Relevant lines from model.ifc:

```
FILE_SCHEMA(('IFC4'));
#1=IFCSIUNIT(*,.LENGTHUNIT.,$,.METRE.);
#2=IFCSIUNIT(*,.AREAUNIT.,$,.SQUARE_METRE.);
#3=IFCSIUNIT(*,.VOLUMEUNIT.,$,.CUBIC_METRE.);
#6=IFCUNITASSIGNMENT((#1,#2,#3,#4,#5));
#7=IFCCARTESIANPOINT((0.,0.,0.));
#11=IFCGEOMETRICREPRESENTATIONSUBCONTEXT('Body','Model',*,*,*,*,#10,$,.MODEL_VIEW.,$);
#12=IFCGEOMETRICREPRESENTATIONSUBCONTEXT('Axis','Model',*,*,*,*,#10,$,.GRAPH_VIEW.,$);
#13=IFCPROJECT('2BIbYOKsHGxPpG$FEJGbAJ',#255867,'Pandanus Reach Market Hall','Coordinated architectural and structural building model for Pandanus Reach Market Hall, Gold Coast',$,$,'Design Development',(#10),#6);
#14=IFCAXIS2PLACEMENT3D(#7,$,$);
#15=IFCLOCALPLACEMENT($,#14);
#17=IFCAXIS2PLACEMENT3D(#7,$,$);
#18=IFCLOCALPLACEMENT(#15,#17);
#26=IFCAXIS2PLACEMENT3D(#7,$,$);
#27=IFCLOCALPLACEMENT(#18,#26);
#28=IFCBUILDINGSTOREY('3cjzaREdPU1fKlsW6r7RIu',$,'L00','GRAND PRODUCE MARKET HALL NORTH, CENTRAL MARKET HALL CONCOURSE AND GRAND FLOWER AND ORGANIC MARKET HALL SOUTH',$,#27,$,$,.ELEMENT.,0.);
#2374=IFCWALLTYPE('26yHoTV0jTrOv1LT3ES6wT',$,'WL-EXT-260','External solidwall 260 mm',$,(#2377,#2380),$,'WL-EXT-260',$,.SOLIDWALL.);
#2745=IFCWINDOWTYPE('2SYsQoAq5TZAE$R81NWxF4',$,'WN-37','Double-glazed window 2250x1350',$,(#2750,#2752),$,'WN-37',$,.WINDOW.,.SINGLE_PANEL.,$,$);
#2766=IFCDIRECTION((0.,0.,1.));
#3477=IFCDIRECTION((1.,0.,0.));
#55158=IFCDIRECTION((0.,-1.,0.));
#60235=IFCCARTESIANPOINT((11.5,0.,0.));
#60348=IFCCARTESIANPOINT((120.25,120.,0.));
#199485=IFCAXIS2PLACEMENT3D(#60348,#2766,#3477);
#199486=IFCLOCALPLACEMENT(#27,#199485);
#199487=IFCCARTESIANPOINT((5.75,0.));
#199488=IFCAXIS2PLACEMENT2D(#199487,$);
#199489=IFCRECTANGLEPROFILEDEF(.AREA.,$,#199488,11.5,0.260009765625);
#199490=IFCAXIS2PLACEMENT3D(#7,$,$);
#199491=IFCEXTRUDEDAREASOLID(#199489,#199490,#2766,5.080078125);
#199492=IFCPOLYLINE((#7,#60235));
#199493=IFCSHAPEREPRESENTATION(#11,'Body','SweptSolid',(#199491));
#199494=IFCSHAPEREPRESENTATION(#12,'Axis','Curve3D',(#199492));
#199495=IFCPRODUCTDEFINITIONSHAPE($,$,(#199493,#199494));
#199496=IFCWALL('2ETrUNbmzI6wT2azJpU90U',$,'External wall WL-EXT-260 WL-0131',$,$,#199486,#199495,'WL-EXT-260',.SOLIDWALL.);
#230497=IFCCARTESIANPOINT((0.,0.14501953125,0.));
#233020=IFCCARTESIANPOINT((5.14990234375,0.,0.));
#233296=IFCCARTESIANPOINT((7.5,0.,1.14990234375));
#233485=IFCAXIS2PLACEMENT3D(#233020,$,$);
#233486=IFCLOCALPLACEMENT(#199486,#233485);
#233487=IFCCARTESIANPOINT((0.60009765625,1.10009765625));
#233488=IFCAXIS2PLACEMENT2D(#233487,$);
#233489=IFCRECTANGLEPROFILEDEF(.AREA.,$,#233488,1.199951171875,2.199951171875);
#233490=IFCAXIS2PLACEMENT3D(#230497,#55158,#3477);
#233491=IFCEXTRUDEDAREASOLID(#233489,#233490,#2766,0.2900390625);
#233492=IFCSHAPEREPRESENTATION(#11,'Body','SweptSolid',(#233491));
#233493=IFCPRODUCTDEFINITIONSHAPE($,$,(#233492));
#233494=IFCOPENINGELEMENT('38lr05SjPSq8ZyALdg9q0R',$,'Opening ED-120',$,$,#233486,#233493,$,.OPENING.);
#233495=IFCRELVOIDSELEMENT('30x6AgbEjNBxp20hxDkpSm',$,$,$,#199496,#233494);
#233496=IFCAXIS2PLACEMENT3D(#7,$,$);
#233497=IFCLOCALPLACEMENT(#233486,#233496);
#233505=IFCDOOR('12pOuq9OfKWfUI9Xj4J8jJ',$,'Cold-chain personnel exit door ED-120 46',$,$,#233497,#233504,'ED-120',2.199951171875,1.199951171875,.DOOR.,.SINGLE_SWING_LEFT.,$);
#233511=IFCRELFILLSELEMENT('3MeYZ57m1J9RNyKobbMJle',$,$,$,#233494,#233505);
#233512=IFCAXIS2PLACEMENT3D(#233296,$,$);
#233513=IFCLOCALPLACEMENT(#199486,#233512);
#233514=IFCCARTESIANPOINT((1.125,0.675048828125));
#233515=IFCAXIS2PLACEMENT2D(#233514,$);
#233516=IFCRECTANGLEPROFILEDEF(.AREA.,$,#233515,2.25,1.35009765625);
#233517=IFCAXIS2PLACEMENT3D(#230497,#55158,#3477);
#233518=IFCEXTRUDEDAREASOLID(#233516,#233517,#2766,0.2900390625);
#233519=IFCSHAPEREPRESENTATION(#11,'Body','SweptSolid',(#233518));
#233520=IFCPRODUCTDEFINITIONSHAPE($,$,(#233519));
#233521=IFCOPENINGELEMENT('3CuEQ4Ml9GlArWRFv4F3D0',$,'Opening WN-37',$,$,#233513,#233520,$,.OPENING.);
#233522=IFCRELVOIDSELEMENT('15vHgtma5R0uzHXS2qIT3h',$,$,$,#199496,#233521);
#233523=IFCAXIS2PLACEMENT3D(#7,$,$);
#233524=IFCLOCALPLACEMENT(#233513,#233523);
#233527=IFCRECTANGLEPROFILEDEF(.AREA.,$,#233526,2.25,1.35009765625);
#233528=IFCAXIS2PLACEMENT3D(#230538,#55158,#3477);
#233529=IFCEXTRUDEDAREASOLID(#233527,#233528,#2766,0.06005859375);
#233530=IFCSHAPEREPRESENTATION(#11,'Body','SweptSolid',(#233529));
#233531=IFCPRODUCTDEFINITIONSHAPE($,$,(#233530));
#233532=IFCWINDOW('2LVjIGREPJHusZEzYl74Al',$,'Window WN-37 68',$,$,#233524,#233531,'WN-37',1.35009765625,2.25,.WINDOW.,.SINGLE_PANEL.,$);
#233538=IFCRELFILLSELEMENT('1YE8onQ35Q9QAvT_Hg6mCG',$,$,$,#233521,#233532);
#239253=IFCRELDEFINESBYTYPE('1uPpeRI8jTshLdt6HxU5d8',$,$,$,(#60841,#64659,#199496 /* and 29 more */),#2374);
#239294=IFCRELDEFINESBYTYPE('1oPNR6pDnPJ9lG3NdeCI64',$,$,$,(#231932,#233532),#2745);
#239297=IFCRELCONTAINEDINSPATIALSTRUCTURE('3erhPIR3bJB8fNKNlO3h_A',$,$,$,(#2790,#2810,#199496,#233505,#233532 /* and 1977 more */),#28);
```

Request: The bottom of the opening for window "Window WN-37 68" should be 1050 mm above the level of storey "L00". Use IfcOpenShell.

```python
import numpy as np
import ifcopenshell
import ifcopenshell.api.geometry
import ifcopenshell.geom
import ifcopenshell.util.element
import ifcopenshell.util.placement
import ifcopenshell.util.shape
import ifcopenshell.util.unit

model = ifcopenshell.open("model.ifc")
unit_scale = ifcopenshell.util.unit.calculate_unit_scale(model)

window = model.by_guid("2LVjIGREPJHusZEzYl74Al")
opening = window.FillsVoids[0].RelatingOpeningElement
storey = ifcopenshell.util.element.get_container(window, ifc_class="IfcBuildingStorey")
level = ifcopenshell.util.placement.get_local_placement(storey.ObjectPlacement)[2, 3]

# The opening's origin need not be at the sill, so measure its lowest point.
shape = ifcopenshell.geom.create_shape(ifcopenshell.geom.settings(), opening)
bottom = ifcopenshell.util.shape.get_shape_bottom_elevation(shape, shape.geometry) / unit_scale
dz = level + 1.05 / unit_scale - bottom

shift = np.array([0.0, 0.0, dz])
# The window is placed relative to its opening, so it follows when the opening moves.
matrix = ifcopenshell.util.placement.get_local_placement(opening.ObjectPlacement)
matrix[:3, 3] += shift
ifcopenshell.api.geometry.edit_object_placement(
    model, product=opening, matrix=matrix, is_si=False, should_transform_children=True
)

print(f"moved by {dz * unit_scale:+.3f} m")

model.write("model_v2.ifc")
```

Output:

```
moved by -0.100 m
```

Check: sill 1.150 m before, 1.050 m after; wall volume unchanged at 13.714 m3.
